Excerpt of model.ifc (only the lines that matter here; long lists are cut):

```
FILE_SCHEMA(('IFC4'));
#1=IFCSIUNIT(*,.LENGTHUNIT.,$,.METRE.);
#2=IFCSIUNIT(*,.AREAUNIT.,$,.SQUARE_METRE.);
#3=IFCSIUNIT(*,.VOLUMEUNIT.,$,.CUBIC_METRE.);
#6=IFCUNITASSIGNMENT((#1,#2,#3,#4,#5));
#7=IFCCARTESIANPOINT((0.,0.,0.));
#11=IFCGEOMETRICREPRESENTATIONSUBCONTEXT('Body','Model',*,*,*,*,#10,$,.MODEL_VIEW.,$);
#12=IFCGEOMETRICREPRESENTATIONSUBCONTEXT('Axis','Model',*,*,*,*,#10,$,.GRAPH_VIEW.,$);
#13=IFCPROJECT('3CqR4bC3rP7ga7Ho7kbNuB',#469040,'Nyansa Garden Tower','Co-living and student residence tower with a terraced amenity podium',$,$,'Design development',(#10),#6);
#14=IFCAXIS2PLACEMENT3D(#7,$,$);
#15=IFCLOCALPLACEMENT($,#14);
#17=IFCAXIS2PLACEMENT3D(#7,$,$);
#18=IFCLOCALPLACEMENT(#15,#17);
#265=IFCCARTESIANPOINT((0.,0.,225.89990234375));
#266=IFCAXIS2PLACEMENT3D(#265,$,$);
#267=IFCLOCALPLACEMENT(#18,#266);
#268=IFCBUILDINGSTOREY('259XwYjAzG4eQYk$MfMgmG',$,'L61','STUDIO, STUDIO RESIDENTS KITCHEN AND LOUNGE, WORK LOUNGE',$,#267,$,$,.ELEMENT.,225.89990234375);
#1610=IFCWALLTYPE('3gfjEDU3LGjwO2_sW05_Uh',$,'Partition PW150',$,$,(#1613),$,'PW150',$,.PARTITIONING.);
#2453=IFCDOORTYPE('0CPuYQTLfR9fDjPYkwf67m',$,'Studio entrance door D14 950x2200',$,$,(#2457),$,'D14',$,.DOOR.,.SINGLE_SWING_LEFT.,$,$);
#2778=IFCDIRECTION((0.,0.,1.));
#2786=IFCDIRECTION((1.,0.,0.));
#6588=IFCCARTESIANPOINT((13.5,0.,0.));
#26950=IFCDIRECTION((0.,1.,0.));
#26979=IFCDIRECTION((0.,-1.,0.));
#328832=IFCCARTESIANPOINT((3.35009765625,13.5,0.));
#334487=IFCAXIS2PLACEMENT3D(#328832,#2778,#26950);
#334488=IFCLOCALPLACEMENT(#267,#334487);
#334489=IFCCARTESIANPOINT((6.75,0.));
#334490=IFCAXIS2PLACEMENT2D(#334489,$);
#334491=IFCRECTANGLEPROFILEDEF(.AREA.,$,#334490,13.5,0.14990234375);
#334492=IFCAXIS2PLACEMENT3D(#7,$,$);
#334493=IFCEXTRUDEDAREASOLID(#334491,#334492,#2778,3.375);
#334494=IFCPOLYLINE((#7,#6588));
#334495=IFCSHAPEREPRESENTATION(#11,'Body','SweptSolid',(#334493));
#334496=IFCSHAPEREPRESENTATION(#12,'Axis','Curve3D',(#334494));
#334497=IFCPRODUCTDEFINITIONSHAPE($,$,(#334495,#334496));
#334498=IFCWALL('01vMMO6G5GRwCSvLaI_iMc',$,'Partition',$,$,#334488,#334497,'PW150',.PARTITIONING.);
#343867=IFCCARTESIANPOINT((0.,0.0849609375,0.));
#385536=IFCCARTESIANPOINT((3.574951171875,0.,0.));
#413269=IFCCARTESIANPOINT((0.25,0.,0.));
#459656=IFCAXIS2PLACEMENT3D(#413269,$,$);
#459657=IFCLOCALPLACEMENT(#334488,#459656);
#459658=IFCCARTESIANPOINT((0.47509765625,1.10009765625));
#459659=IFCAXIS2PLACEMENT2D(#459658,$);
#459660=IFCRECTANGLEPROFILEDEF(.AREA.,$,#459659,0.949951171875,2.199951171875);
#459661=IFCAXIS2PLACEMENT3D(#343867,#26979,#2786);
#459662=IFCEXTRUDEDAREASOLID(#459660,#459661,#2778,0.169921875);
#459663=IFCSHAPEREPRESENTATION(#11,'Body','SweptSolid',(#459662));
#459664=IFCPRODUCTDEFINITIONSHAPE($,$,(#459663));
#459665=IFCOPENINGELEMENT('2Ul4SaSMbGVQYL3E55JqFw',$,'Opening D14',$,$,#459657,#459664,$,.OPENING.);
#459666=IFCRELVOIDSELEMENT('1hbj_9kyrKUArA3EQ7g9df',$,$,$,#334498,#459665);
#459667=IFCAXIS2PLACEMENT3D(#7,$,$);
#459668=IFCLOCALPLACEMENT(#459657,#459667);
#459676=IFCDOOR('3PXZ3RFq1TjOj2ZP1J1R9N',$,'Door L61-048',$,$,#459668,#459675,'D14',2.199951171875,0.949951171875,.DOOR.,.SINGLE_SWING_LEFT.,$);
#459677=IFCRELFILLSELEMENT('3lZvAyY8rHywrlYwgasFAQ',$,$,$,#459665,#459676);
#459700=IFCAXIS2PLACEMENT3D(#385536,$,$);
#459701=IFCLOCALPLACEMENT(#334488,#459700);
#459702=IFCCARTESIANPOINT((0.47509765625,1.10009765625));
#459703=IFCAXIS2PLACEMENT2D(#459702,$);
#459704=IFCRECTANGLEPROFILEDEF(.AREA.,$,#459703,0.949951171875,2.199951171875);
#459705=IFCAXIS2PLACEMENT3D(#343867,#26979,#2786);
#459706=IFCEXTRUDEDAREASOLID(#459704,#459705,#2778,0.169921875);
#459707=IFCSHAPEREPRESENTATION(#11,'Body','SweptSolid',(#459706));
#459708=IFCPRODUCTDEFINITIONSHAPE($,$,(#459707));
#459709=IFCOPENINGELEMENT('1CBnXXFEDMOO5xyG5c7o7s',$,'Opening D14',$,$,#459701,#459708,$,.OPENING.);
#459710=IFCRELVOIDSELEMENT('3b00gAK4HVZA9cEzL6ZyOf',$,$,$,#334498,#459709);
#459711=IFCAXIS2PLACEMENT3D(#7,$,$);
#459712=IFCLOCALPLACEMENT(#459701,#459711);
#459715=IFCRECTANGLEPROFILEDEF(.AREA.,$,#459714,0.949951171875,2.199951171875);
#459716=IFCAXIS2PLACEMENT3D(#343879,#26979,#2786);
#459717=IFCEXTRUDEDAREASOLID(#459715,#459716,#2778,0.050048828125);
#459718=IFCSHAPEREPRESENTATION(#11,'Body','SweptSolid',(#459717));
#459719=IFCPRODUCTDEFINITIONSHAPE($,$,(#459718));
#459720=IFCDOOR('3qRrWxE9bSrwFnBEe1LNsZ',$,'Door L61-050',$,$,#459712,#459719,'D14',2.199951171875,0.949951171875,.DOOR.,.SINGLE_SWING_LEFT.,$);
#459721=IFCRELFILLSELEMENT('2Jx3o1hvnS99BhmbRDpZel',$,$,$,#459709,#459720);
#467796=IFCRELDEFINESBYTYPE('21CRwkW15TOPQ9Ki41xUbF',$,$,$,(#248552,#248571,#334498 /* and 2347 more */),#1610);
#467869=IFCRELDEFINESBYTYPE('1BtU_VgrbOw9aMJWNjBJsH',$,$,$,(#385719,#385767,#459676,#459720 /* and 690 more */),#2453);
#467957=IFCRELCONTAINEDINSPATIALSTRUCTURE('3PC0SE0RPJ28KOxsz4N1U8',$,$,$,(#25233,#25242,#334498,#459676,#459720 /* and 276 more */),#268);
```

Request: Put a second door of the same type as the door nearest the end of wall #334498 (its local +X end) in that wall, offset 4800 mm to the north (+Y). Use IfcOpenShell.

```python
import ifcopenshell
import ifcopenshell.api.feature
import ifcopenshell.api.geometry
import ifcopenshell.api.root
import ifcopenshell.geom
import ifcopenshell.util.element
import ifcopenshell.util.placement
import ifcopenshell.util.shape

model = ifcopenshell.open("model.ifc")
settings = ifcopenshell.geom.settings()


def volume(element):
    """Net volume in cubic metres, openings subtracted."""
    shape = ifcopenshell.geom.create_shape(settings, element)
    return ifcopenshell.util.shape.get_volume(shape.geometry)


door = model.by_guid("3qRrWxE9bSrwFnBEe1LNsZ")
opening = door.FillsVoids[0].RelatingOpeningElement
wall = opening.VoidsElements[0].RelatingBuildingElement
before = volume(wall)
shift = ifcopenshell.util.placement.get_local_placement(wall.ObjectPlacement)[:3, 0] * 4.8

# copy_class copies the void relationship, type, container and properties, but no geometry.
new_opening = ifcopenshell.api.root.copy_class(model, product=opening)
new_opening.Representation = ifcopenshell.util.element.copy_deep(
    model, opening.Representation, exclude=["IfcGeometricRepresentationContext", "IfcRepresentationMap"]
)
new_door = ifcopenshell.api.root.copy_class(model, product=door)
new_door.Representation = ifcopenshell.util.element.copy_deep(
    model, door.Representation, exclude=["IfcGeometricRepresentationContext", "IfcRepresentationMap"]
)
new_door.Tag = None
ifcopenshell.api.feature.add_filling(model, opening=new_opening, element=new_door)

for old, new in ((opening, new_opening), (door, new_door)):
    matrix = ifcopenshell.util.placement.get_local_placement(old.ObjectPlacement)
    matrix[:3, 3] += shift
    ifcopenshell.api.geometry.edit_object_placement(model, product=new, matrix=matrix, is_si=False)

after = volume(wall)

print(f"wall volume {before:.3f} -> {after:.3f} m3")

model.write("model_updated.ifc")
```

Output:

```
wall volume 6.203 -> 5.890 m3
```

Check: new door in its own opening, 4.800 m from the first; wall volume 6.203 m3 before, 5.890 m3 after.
